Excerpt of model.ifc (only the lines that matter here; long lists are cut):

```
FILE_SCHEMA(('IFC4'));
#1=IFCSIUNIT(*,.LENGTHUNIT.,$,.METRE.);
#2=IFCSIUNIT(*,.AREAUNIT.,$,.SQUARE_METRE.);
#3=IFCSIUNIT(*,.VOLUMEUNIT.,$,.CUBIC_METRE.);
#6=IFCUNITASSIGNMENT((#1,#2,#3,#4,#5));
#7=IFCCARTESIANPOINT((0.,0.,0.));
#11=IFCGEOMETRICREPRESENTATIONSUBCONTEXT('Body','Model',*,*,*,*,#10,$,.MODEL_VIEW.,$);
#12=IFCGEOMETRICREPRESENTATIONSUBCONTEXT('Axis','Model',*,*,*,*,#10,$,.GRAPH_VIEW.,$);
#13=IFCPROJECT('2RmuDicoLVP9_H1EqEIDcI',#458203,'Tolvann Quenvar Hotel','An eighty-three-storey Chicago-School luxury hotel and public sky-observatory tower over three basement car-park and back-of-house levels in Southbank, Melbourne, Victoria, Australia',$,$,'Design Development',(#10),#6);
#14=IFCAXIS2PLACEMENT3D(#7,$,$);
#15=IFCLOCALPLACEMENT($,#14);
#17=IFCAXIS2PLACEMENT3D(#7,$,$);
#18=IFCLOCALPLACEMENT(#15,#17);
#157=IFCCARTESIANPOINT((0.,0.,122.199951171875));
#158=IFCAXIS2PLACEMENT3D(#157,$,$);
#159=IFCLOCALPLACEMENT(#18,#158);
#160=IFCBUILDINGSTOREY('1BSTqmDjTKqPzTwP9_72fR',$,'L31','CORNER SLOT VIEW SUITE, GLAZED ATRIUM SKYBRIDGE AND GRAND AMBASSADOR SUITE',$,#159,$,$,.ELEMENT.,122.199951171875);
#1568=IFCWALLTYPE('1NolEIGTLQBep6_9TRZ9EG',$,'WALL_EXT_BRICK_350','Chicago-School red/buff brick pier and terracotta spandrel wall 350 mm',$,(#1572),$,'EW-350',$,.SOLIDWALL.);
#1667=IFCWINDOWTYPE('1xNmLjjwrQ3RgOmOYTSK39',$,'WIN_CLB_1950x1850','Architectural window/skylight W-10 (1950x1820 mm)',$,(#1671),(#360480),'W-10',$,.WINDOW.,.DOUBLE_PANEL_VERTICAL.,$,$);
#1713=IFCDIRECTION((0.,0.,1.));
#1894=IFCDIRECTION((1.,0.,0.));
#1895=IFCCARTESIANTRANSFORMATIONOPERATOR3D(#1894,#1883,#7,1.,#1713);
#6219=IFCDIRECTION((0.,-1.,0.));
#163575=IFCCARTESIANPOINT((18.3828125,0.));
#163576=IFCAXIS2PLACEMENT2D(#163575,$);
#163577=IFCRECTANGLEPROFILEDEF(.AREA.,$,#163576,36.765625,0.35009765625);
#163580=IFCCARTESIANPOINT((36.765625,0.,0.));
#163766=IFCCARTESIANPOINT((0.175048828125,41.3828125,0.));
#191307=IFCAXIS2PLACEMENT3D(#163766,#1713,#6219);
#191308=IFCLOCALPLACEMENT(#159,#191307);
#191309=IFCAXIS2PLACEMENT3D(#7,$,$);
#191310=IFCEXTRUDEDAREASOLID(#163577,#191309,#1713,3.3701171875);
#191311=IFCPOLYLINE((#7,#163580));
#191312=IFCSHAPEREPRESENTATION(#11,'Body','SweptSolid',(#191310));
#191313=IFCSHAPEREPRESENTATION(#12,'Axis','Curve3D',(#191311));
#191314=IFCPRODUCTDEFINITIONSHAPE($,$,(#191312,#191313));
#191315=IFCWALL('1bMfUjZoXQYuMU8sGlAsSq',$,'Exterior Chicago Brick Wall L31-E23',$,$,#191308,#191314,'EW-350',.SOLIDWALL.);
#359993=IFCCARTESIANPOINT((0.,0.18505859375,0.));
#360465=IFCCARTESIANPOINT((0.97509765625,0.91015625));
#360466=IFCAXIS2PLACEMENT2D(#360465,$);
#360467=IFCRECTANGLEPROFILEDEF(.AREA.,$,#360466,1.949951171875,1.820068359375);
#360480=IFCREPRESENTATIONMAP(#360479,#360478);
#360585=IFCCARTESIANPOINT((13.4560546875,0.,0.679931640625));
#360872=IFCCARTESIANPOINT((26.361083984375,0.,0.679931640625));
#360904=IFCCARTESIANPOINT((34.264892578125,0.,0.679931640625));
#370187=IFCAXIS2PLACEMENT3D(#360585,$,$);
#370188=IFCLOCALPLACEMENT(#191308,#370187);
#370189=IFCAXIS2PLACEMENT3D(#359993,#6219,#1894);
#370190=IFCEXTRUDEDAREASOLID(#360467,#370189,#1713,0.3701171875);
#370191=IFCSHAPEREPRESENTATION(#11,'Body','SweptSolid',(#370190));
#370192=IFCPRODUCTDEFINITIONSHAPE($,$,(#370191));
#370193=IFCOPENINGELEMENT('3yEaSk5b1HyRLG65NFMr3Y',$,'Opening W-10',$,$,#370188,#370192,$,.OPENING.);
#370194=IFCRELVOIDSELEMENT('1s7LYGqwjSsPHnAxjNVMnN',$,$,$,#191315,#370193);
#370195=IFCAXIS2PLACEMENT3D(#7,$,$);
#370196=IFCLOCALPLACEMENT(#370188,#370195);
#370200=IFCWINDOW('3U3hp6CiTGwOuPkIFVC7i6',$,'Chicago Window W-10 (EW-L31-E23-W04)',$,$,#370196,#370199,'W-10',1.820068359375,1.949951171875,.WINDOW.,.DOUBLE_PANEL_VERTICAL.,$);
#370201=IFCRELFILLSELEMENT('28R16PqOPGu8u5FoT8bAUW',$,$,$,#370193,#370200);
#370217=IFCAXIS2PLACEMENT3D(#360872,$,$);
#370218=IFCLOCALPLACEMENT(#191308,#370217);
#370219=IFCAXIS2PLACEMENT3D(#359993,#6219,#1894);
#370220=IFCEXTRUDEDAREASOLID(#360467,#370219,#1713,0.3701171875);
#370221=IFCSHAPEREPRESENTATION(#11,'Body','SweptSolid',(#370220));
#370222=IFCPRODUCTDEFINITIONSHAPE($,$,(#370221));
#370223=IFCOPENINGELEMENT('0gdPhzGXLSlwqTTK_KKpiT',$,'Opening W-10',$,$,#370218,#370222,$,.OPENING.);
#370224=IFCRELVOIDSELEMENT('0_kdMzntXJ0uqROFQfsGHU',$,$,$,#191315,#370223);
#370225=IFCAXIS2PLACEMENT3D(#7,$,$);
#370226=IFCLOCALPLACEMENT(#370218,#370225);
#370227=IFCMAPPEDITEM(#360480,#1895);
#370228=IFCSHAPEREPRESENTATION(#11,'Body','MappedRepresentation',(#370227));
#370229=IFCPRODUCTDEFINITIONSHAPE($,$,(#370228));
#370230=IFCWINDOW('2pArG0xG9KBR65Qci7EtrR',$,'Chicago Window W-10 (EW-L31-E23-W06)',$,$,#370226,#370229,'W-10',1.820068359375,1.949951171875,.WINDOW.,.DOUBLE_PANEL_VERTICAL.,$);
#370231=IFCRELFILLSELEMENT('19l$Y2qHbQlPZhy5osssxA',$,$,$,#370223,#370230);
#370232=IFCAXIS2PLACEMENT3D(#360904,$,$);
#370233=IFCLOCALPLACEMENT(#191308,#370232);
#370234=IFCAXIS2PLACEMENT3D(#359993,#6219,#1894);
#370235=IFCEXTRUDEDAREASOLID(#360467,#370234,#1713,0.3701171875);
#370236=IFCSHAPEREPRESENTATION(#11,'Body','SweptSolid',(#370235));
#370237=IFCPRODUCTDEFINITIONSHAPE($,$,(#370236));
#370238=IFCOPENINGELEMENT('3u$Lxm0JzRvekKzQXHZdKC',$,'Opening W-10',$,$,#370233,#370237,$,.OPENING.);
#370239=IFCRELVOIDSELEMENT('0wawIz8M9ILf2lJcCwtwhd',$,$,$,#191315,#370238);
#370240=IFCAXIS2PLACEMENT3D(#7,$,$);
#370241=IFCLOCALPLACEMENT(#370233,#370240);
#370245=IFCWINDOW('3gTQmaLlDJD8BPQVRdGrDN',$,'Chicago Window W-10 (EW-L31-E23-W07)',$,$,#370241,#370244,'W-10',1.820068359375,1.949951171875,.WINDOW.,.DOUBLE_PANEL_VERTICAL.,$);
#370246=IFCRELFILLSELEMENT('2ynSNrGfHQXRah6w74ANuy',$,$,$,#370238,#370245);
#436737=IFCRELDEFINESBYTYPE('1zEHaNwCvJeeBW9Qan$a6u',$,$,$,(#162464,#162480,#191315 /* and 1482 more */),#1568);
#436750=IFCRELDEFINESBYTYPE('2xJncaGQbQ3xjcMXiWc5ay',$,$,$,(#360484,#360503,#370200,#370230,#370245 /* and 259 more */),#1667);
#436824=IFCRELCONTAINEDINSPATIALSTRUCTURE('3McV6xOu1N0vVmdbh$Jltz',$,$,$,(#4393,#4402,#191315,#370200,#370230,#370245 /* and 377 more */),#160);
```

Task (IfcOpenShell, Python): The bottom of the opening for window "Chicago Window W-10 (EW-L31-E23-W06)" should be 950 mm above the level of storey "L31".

```python
import numpy as np
import ifcopenshell
import ifcopenshell.api.geometry
import ifcopenshell.geom
import ifcopenshell.util.element
import ifcopenshell.util.placement
import ifcopenshell.util.shape
import ifcopenshell.util.unit

model = ifcopenshell.open("model.ifc")
unit_scale = ifcopenshell.util.unit.calculate_unit_scale(model)

window = model.by_guid("2pArG0xG9KBR65Qci7EtrR")
opening = window.FillsVoids[0].RelatingOpeningElement
storey = ifcopenshell.util.element.get_container(window, ifc_class="IfcBuildingStorey")
level = ifcopenshell.util.placement.get_local_placement(storey.ObjectPlacement)[2, 3]

# The opening's origin need not be at the sill, so measure its lowest point.
shape = ifcopenshell.geom.create_shape(ifcopenshell.geom.settings(), opening)
bottom = ifcopenshell.util.shape.get_shape_bottom_elevation(shape, shape.geometry) / unit_scale
dz = level + 0.95 / unit_scale - bottom

shift = np.array([0.0, 0.0, dz])
# The window is placed relative to its opening, so it follows when the opening moves.
matrix = ifcopenshell.util.placement.get_local_placement(opening.ObjectPlacement)
matrix[:3, 3] += shift
ifcopenshell.api.geometry.edit_object_placement(
    model, product=opening, matrix=matrix, is_si=False, should_transform_children=True
)

print(f"moved by {dz * unit_scale:+.3f} m")

model.write("model-out.ifc")
```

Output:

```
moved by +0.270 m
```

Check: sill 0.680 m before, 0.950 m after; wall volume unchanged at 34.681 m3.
